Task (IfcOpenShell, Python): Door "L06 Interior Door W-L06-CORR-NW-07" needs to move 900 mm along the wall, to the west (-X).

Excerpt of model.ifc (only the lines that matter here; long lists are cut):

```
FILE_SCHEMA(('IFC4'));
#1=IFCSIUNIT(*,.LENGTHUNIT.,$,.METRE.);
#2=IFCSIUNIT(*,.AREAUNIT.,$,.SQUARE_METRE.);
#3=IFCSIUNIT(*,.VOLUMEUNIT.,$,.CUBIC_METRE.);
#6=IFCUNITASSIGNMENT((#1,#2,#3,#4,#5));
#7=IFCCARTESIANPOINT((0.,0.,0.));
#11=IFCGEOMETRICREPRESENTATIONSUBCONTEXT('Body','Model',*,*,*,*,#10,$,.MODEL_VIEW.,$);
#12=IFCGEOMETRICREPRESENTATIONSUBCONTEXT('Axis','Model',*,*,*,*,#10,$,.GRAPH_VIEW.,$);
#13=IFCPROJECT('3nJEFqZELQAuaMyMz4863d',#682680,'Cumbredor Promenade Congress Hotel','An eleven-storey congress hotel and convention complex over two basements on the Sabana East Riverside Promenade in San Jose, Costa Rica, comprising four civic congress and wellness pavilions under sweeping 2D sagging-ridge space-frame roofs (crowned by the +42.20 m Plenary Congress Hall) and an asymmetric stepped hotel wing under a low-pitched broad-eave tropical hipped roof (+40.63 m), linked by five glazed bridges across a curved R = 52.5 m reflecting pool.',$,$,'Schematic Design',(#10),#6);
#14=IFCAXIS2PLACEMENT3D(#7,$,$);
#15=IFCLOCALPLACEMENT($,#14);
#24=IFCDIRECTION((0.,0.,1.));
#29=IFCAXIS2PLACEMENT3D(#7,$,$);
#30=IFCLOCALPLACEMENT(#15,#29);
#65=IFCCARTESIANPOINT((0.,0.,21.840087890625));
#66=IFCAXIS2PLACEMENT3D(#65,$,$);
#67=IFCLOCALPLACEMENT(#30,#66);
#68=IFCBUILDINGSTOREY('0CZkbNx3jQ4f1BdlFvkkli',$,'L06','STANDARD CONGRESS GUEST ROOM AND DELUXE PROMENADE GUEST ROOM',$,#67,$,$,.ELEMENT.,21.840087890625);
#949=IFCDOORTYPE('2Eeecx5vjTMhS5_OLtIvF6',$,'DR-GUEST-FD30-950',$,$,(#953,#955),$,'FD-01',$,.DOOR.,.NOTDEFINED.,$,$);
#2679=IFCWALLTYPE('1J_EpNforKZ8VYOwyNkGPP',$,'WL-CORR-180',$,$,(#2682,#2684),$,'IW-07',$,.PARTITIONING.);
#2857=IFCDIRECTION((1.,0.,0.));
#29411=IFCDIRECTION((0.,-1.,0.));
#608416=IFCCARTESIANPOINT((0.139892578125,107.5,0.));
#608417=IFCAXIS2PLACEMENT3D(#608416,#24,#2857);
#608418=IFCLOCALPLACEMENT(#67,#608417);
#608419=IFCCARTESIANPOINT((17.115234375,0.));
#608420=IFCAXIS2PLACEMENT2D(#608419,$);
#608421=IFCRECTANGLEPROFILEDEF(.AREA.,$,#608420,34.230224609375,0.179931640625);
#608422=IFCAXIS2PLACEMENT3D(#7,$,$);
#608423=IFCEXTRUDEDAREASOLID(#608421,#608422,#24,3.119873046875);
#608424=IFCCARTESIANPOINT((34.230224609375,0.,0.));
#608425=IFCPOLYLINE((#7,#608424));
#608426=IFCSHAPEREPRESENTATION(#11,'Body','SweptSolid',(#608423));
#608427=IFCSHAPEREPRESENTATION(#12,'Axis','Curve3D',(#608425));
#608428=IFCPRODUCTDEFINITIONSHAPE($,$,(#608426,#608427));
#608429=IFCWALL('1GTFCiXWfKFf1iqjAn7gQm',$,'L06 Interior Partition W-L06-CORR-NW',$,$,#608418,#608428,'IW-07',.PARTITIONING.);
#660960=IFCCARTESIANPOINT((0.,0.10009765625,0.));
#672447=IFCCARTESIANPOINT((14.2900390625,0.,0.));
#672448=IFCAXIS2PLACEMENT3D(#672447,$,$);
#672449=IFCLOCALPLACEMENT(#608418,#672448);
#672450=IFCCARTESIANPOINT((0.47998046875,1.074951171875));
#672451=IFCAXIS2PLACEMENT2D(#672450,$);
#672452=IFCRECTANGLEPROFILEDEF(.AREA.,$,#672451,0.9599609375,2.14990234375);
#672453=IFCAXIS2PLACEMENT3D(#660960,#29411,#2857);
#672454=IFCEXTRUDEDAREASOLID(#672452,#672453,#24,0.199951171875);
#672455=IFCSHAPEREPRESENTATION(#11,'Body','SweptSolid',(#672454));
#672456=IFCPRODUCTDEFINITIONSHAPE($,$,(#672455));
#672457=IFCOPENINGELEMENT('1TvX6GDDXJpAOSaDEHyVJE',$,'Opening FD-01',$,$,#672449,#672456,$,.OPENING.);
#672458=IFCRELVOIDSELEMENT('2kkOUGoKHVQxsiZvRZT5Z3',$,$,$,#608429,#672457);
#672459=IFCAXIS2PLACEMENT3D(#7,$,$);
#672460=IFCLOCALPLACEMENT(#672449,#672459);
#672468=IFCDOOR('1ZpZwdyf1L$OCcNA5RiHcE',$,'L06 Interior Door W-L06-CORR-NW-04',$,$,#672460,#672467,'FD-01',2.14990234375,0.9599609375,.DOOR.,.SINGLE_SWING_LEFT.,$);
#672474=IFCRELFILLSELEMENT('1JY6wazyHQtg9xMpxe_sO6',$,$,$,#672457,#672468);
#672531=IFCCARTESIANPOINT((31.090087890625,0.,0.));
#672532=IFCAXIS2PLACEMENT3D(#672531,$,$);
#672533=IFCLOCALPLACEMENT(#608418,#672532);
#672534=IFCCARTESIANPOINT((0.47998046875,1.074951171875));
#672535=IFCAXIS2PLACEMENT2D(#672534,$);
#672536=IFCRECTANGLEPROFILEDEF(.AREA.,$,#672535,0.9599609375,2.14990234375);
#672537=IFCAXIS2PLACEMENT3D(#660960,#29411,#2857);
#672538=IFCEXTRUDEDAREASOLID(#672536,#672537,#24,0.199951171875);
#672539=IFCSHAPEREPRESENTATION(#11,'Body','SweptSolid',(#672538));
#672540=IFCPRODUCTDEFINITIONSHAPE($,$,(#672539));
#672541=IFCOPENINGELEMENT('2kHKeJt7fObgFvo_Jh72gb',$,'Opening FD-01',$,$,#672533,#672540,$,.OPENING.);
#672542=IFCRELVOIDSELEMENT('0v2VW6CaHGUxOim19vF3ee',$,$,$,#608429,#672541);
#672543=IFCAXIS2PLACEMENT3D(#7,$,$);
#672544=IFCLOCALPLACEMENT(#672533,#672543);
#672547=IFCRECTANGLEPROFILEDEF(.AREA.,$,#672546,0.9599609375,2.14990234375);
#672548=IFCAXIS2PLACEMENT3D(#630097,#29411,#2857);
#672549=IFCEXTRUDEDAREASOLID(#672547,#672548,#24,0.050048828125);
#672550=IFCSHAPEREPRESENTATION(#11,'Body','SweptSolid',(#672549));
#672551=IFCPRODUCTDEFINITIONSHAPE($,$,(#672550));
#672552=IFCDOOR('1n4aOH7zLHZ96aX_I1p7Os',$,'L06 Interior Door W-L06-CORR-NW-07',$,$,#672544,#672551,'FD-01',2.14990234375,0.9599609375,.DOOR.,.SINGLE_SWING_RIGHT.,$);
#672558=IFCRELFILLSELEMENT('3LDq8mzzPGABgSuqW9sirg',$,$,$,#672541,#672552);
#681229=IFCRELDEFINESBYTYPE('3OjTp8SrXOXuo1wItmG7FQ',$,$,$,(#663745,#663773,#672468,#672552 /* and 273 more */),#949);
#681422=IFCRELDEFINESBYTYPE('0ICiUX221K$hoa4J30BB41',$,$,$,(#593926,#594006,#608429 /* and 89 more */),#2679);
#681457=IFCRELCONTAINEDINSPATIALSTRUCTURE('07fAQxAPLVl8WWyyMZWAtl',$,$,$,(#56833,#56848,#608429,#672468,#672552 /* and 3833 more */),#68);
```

```python
import ifcopenshell
import ifcopenshell.api.geometry
import ifcopenshell.util.placement
import ifcopenshell.util.unit

model = ifcopenshell.open("model.ifc")
unit_scale = ifcopenshell.util.unit.calculate_unit_scale(model)

door = model.by_guid("1n4aOH7zLHZ96aX_I1p7Os")
opening = door.FillsVoids[0].RelatingOpeningElement
wall = opening.VoidsElements[0].RelatingBuildingElement

wall_matrix = ifcopenshell.util.placement.get_local_placement(wall.ObjectPlacement)
shift = wall_matrix[:3, 0] * -0.9 / unit_scale
before = ifcopenshell.util.placement.get_local_placement(door.ObjectPlacement)[:3, 3].copy()

# The door is placed relative to its opening, so it follows when the opening moves.
matrix = ifcopenshell.util.placement.get_local_placement(opening.ObjectPlacement)
matrix[:3, 3] += shift
ifcopenshell.api.geometry.edit_object_placement(
    model, product=opening, matrix=matrix, is_si=False, should_transform_children=True
)

after = ifcopenshell.util.placement.get_local_placement(door.ObjectPlacement)[:3, 3]
print("door moved by", (after - before).round(3) + 0.0)

model.write("model_v2.ifc")
```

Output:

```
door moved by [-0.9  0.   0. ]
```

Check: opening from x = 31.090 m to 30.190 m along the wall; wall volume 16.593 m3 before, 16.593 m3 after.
